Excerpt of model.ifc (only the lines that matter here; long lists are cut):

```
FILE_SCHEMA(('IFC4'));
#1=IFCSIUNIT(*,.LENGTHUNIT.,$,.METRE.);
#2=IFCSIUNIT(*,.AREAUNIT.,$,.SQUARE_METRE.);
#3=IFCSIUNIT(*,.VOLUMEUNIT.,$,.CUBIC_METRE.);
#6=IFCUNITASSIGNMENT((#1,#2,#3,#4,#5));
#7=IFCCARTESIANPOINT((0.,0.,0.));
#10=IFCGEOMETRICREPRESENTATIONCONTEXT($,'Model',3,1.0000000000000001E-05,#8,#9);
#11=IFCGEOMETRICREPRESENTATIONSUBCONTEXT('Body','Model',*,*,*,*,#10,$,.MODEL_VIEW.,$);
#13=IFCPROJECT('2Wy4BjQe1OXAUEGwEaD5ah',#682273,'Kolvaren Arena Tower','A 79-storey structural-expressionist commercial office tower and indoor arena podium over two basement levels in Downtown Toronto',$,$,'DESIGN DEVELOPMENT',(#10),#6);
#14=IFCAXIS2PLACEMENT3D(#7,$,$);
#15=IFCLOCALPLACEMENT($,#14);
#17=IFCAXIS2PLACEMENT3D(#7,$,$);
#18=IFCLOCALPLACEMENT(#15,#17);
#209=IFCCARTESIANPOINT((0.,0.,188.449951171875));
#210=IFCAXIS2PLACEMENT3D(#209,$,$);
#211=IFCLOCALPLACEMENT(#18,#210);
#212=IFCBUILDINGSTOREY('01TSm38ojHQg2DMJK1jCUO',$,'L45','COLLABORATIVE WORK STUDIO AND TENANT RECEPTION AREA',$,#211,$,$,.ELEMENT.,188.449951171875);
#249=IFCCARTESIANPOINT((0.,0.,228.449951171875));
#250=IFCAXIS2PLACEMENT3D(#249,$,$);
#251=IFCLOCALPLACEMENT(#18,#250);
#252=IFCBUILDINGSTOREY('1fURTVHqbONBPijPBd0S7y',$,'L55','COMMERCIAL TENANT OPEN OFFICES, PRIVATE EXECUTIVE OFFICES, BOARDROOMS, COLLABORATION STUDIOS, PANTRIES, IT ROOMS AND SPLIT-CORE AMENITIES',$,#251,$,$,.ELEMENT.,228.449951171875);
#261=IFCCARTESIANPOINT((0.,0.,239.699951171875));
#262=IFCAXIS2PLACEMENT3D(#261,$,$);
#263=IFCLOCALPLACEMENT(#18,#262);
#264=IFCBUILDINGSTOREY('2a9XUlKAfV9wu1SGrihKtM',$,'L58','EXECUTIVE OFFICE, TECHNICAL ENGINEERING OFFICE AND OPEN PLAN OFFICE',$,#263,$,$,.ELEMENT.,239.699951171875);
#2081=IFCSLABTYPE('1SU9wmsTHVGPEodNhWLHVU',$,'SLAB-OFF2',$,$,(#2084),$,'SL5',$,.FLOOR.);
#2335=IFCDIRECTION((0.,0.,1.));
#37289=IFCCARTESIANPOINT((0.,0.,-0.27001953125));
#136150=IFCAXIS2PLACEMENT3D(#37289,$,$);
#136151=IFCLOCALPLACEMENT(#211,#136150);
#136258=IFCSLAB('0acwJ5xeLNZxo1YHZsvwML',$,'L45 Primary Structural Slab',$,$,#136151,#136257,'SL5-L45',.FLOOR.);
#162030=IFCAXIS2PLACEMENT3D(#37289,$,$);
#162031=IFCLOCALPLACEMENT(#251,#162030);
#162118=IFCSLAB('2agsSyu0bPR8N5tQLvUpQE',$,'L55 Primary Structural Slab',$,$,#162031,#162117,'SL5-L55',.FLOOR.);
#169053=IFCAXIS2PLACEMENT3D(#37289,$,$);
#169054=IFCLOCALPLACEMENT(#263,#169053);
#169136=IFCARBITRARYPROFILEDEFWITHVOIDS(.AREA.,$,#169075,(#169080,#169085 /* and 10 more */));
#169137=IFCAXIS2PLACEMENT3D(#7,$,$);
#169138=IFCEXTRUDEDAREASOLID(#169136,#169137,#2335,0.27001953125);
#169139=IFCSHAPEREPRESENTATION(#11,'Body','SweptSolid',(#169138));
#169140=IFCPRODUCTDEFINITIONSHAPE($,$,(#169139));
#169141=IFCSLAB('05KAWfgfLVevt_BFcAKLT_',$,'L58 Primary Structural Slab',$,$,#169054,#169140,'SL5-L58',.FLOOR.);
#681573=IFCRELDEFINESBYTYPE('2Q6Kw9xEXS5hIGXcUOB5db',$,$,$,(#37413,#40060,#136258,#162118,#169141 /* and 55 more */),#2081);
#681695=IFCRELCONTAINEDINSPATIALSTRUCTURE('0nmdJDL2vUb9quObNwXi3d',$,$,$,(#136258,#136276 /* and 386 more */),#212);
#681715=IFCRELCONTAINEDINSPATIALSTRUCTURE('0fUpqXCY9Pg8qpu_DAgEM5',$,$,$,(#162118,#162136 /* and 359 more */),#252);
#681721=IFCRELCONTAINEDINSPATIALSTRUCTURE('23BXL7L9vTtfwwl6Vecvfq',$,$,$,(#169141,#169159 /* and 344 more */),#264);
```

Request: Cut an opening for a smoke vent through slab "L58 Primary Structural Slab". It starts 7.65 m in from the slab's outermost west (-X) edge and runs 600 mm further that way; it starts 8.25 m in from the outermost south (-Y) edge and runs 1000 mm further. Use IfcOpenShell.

```python
import numpy as np
import ifcopenshell
import ifcopenshell.api.feature
import ifcopenshell.api.geometry
import ifcopenshell.api.root
import ifcopenshell.geom
import ifcopenshell.util.placement
import ifcopenshell.util.representation
import ifcopenshell.util.shape
import ifcopenshell.util.unit

model = ifcopenshell.open("model.ifc")
unit_scale = ifcopenshell.util.unit.calculate_unit_scale(model)
settings = ifcopenshell.geom.settings()


def volume(element):
    """Net volume in cubic metres, openings subtracted."""
    shape = ifcopenshell.geom.create_shape(settings, element)
    return ifcopenshell.util.shape.get_volume(shape.geometry)


slab = model.by_guid("05KAWfgfLVevt_BFcAKLT_")
before = volume(slab)

# Extent in the slab's own axes, in metres. The edges named are its -X and -Y sides.
slab_shape = ifcopenshell.geom.create_shape(settings, slab)
vertices = ifcopenshell.util.shape.get_vertices(slab_shape.geometry)
x_min, y_min, bottom = vertices.min(axis=0)
top = vertices[:, 2].max()

opening = ifcopenshell.api.root.create_entity(model, ifc_class="IfcOpeningElement", name="Smoke vent opening", predefined_type="OPENING")
context = ifcopenshell.util.representation.get_context(model, "Model", "Body", "MODEL_VIEW")
width, depth = 0.6, 1
outline = [(0.0, 0.0), (width, 0.0), (width, depth), (0.0, depth), (0.0, 0.0)]
# Overshoot both faces by 50 mm so the cut is clean.
shape = ifcopenshell.api.geometry.add_slab_representation(
    model, context=context, depth=top - bottom + 0.1, polyline=outline
)
ifcopenshell.api.geometry.assign_representation(model, product=opening, representation=shape)

matrix = ifcopenshell.util.placement.get_local_placement(slab.ObjectPlacement)
matrix[:, 3] = matrix @ np.append(np.array([x_min + 7.65, y_min + 8.25, bottom - 0.05]) / unit_scale, 1.0)
ifcopenshell.api.geometry.edit_object_placement(model, product=opening, matrix=matrix, is_si=False)
ifcopenshell.api.feature.add_feature(model, feature=opening, element=slab)

after = volume(slab)

print(f"slab volume {before:.3f} -> {after:.3f} m3")

model.write("model_rev.ifc")
```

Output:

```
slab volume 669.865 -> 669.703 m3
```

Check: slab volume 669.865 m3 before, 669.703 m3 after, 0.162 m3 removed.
